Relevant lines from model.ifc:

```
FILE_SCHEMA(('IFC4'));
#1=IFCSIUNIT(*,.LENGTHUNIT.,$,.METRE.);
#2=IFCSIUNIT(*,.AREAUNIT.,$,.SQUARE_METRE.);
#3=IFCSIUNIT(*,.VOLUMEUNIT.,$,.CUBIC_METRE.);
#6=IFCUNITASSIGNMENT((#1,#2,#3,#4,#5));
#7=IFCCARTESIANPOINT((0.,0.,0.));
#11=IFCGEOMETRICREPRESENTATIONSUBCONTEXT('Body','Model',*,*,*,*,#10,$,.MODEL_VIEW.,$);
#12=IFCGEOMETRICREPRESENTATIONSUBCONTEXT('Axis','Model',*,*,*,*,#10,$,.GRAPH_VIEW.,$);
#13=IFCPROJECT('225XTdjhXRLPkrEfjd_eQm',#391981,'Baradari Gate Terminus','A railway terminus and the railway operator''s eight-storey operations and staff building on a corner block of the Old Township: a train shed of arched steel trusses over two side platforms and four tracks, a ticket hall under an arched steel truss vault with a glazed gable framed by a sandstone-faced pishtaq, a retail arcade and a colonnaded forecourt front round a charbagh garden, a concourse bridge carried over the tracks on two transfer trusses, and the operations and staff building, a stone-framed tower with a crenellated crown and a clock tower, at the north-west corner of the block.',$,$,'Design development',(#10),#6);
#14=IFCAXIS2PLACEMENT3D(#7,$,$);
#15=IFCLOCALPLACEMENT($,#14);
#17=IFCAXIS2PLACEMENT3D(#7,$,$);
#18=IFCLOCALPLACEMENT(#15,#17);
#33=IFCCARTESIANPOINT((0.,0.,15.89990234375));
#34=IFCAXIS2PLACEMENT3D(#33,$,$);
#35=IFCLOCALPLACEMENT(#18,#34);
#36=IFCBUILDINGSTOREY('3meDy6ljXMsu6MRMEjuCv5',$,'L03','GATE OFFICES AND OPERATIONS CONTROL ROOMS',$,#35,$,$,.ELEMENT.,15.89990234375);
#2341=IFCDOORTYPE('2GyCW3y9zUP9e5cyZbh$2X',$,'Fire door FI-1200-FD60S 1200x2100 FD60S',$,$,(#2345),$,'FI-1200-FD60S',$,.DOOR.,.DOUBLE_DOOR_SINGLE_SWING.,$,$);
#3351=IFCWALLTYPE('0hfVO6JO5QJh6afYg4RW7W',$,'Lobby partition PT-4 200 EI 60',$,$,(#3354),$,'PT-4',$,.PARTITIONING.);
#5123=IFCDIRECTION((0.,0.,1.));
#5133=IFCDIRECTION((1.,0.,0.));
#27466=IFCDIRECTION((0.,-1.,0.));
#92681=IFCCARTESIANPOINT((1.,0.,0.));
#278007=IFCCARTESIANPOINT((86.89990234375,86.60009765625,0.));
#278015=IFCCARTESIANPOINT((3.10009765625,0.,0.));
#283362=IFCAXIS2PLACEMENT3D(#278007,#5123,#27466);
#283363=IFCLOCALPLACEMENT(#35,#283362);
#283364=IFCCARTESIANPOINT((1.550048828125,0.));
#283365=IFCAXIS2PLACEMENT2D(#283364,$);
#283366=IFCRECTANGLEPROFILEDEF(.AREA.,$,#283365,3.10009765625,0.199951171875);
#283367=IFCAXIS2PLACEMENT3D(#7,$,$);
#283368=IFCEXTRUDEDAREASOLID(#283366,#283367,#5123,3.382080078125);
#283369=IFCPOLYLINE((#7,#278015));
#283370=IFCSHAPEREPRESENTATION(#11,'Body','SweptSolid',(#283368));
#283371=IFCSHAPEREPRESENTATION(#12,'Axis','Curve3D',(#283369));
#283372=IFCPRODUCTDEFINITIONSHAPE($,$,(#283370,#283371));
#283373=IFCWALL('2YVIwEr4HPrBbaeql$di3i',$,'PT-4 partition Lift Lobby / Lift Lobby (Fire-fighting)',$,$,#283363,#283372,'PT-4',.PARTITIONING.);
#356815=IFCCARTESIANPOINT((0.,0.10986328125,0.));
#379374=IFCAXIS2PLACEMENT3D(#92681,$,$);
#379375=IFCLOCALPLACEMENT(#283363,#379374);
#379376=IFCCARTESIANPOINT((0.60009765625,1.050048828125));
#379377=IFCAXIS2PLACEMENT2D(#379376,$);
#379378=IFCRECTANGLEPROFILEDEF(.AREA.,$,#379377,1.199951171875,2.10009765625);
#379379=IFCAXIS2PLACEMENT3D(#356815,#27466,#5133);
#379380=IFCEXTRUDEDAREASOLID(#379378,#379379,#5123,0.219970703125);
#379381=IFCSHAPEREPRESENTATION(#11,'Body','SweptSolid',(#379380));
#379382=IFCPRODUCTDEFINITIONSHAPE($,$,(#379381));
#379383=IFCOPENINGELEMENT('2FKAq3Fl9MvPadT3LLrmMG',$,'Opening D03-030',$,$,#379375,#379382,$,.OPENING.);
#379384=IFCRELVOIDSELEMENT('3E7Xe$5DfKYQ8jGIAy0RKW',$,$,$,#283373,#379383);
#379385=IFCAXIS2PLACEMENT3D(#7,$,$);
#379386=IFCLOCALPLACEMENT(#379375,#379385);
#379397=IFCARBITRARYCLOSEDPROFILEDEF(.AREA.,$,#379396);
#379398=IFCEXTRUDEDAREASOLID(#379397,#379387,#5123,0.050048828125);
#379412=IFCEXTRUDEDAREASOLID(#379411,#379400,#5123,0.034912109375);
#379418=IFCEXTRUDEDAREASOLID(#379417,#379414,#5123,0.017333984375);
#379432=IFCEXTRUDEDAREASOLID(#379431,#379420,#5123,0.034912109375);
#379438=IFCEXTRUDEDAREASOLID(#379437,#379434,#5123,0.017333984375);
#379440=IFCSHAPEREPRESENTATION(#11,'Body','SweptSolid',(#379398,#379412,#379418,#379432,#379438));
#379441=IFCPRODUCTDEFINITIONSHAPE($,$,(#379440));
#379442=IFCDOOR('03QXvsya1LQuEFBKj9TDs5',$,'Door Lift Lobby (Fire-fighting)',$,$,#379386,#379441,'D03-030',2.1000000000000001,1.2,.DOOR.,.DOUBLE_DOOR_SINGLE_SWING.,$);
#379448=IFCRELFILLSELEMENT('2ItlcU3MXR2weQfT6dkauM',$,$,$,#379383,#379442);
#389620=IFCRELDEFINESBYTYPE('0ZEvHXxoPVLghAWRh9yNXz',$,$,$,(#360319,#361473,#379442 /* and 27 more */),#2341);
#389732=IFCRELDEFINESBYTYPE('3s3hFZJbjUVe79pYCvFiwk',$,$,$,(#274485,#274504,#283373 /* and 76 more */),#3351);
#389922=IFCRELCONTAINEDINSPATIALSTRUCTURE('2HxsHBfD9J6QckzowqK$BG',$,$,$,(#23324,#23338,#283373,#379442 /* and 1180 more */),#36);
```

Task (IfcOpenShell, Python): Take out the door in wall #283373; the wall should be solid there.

```python
import ifcopenshell
import ifcopenshell.api.feature
import ifcopenshell.api.root
import ifcopenshell.geom
import ifcopenshell.util.shape

model = ifcopenshell.open("model.ifc")
settings = ifcopenshell.geom.settings()


def volume(element):
    """Net volume in cubic metres, openings subtracted."""
    shape = ifcopenshell.geom.create_shape(settings, element)
    return ifcopenshell.util.shape.get_volume(shape.geometry)


door = model.by_id(379442)
opening = door.FillsVoids[0].RelatingOpeningElement
wall = opening.VoidsElements[0].RelatingBuildingElement
before = volume(wall)

ifcopenshell.api.root.remove_product(model, product=door)
ifcopenshell.api.feature.remove_feature(model, feature=opening)

after = volume(wall)

print(f"wall volume {before:.3f} -> {after:.3f} m3")

model.write("model_updated.ifc")
```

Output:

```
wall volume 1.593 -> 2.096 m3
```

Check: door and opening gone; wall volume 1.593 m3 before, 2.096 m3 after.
